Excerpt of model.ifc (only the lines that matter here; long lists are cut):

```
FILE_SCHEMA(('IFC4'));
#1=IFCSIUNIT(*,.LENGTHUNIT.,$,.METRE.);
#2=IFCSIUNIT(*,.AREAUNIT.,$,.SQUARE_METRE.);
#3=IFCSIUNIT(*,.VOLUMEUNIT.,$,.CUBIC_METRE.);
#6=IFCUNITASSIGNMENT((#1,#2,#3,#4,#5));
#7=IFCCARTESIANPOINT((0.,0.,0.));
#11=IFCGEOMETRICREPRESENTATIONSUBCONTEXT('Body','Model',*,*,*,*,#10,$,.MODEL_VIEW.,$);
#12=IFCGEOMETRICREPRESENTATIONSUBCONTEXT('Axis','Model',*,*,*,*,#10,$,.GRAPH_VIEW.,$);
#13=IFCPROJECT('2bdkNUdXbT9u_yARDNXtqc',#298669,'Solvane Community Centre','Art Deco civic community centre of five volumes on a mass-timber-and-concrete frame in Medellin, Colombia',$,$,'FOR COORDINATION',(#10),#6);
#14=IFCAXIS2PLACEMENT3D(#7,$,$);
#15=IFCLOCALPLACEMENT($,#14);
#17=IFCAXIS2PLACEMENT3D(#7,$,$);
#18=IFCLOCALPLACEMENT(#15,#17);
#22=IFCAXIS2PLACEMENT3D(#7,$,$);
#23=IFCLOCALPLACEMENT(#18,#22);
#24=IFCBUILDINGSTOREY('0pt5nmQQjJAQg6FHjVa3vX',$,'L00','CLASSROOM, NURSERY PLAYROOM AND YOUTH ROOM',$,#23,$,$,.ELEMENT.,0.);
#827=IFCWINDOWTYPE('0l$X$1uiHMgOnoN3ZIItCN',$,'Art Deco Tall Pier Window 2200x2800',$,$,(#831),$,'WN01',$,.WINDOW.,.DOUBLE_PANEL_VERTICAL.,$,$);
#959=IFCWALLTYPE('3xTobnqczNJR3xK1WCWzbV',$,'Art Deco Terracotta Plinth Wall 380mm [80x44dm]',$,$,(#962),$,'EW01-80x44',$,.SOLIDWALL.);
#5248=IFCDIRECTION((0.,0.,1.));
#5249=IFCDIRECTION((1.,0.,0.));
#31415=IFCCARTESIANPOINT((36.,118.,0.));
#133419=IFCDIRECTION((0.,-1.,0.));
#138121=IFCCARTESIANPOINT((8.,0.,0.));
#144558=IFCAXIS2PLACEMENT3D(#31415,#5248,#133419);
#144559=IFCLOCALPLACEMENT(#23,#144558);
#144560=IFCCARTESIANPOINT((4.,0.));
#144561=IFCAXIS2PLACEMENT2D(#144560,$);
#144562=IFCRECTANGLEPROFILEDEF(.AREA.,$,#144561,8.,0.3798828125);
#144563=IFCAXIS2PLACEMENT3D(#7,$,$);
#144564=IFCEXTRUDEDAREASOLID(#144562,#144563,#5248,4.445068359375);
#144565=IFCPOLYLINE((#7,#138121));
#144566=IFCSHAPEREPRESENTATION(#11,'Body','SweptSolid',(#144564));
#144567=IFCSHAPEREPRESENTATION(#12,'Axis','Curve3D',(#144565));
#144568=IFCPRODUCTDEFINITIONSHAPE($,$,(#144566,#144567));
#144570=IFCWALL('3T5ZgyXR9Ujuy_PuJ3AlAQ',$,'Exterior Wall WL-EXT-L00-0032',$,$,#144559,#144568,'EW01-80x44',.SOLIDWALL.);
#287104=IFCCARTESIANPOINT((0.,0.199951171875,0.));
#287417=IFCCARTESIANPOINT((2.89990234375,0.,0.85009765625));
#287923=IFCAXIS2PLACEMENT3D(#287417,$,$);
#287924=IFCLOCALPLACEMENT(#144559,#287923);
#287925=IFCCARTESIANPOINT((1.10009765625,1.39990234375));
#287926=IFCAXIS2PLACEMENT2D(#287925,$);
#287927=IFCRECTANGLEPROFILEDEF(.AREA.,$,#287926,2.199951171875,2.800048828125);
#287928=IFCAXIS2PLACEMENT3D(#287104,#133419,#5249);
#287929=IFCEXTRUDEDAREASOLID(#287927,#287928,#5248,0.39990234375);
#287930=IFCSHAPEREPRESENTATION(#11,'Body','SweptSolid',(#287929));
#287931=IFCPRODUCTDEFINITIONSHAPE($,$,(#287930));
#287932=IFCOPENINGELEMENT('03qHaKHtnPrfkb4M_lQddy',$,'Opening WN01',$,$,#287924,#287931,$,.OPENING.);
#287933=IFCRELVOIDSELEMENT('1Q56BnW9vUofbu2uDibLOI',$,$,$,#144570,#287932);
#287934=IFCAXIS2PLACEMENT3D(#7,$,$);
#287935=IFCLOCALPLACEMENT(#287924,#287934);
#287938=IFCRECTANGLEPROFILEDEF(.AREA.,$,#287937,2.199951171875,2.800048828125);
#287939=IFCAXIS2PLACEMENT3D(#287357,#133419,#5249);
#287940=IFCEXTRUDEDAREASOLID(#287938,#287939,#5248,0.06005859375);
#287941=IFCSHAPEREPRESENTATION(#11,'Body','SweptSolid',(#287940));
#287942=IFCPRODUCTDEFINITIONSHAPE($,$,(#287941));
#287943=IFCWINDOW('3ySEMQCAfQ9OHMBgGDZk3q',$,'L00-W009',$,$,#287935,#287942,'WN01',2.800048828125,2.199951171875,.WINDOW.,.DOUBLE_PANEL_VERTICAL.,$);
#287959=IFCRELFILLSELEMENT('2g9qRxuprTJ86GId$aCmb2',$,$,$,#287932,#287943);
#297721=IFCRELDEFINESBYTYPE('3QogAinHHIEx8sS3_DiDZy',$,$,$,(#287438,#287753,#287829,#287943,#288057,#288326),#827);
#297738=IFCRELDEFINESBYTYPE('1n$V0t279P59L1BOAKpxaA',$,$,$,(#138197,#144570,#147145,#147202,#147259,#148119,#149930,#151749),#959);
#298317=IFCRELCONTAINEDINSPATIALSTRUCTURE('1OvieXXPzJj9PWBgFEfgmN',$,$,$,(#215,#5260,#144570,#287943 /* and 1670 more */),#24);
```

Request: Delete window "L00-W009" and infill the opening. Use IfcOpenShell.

```python
import ifcopenshell
import ifcopenshell.api.feature
import ifcopenshell.api.root
import ifcopenshell.geom
import ifcopenshell.util.shape

model = ifcopenshell.open("model.ifc")
settings = ifcopenshell.geom.settings()


def volume(element):
    """Net volume in cubic metres, openings subtracted."""
    shape = ifcopenshell.geom.create_shape(settings, element)
    return ifcopenshell.util.shape.get_volume(shape.geometry)


window = model.by_guid("3ySEMQCAfQ9OHMBgGDZk3q")
opening = window.FillsVoids[0].RelatingOpeningElement
wall = opening.VoidsElements[0].RelatingBuildingElement
before = volume(wall)

ifcopenshell.api.root.remove_product(model, product=window)
ifcopenshell.api.feature.remove_feature(model, feature=opening)

after = volume(wall)

print(f"wall volume {before:.3f} -> {after:.3f} m3")

model.write("model_updated.ifc")
```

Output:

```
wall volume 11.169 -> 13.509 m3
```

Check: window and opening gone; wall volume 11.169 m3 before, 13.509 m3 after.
